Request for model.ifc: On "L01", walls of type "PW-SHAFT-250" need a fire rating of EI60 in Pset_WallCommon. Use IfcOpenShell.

First a look at what the model holds.

```python
import ifcopenshell
import ifcopenshell.util.element

model = ifcopenshell.open("model.ifc")
print(model.schema)
storey = next(s for s in model.by_type("IfcBuildingStorey") if s.Name == "L01")
walls = [e for e in ifcopenshell.util.element.get_decomposition(storey) if e.is_a("IfcWall")]
seen = {}
for e in walls:
    element_type = ifcopenshell.util.element.get_type(e)
    key = (element_type.Name if element_type != e and element_type else None, ifcopenshell.util.element.get_pset(e, "Pset_WallCommon", "FireRating"))
    seen[key] = seen.get(key, 0) + 1
for (name, value), count in sorted(seen.items(), key=str):
    print(count, "x", name, "|", value)
```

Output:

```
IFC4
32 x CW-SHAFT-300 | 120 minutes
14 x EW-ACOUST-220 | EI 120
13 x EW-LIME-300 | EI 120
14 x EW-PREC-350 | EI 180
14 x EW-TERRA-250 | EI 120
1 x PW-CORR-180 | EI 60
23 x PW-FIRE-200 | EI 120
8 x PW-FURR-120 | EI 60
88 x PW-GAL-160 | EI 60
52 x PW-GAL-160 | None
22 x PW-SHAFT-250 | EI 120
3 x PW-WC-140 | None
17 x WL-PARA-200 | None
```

```python
import ifcopenshell
import ifcopenshell.api.pset
import ifcopenshell.util.element

model = ifcopenshell.open("model.ifc")

storey = next(s for s in model.by_type("IfcBuildingStorey") if s.Name == "L01")
walls = [e for e in ifcopenshell.util.element.get_decomposition(storey) if e.is_a("IfcWall")]

count = 0
for e in walls:
    element_type = ifcopenshell.util.element.get_type(e)
    if element_type in (None, e) or element_type.Name != "PW-SHAFT-250":
        continue
    # add_pset returns the element's existing set when there is one.
    pset = ifcopenshell.api.pset.add_pset(model, product=e, name="Pset_WallCommon")
    ifcopenshell.api.pset.edit_pset(model, pset=pset, properties={"FireRating": "EI60"})
    count += 1

print(count, "walls updated")

model.write("model-out.ifc")
```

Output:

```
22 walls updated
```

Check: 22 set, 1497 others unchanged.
